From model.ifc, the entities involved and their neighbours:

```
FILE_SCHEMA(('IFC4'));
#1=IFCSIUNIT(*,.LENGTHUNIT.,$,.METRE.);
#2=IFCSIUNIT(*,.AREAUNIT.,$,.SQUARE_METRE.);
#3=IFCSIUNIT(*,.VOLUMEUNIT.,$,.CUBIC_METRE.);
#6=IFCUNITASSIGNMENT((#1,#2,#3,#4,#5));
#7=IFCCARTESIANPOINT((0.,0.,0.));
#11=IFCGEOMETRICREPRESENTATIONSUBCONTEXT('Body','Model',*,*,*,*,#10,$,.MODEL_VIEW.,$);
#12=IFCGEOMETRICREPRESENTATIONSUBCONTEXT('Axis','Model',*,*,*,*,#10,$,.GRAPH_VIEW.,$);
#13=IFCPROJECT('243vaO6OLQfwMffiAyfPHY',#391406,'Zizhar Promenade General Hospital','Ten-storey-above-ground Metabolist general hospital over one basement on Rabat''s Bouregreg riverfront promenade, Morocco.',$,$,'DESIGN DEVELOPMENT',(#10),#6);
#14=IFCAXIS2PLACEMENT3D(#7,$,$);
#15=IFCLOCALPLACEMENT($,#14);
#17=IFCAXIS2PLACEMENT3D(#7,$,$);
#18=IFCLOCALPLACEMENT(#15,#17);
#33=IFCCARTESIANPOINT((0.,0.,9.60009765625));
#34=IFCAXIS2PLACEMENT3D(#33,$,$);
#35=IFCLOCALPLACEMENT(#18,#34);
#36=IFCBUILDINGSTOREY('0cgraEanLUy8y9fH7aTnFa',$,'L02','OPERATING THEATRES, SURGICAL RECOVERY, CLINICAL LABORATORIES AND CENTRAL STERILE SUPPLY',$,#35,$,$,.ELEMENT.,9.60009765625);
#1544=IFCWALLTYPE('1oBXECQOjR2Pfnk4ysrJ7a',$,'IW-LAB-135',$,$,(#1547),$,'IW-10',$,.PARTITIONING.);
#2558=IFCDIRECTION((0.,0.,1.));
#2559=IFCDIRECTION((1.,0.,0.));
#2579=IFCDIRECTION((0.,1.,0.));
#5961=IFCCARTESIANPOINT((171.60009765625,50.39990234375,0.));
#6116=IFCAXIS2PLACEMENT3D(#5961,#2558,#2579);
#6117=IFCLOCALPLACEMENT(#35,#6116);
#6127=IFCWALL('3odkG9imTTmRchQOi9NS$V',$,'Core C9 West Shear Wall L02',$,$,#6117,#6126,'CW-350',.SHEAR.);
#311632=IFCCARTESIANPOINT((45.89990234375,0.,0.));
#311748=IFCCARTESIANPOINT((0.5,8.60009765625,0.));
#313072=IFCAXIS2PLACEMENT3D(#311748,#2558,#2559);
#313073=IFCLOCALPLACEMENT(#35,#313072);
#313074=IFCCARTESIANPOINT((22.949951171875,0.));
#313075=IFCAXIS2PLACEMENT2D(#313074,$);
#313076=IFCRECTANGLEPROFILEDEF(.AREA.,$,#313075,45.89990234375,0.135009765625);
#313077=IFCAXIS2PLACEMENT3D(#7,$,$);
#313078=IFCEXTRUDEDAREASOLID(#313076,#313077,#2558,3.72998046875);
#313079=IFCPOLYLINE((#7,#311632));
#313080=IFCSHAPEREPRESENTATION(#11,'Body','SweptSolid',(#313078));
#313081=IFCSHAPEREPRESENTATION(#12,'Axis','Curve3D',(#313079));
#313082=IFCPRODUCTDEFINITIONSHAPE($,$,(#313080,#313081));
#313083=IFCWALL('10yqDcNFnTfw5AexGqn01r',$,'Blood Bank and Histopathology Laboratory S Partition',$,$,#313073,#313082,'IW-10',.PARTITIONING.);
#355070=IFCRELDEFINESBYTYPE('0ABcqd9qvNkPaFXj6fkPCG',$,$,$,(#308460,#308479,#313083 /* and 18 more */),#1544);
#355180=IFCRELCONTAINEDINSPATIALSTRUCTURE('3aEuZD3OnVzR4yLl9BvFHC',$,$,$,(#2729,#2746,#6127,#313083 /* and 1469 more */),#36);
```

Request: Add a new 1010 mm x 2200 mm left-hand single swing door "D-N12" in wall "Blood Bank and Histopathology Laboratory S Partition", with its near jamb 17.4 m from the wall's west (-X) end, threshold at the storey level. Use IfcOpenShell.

```python
import numpy as np
import ifcopenshell
import ifcopenshell.api.feature
import ifcopenshell.api.geometry
import ifcopenshell.api.root
import ifcopenshell.api.spatial
import ifcopenshell.geom
import ifcopenshell.util.element
import ifcopenshell.util.placement
import ifcopenshell.util.representation
import ifcopenshell.util.shape
import ifcopenshell.util.unit

model = ifcopenshell.open("model.ifc")
unit_scale = ifcopenshell.util.unit.calculate_unit_scale(model)
settings = ifcopenshell.geom.settings()


def volume(element):
    """Net volume in cubic metres, openings subtracted."""
    shape = ifcopenshell.geom.create_shape(settings, element)
    return ifcopenshell.util.shape.get_volume(shape.geometry)


wall = model.by_guid("10yqDcNFnTfw5AexGqn01r")
storey = ifcopenshell.util.element.get_container(wall, ifc_class="IfcBuildingStorey")
context = ifcopenshell.util.representation.get_context(model, "Model", "Body", "MODEL_VIEW")
before = volume(wall)

width, height, from_end, sill = 1.01, 2.2, 17.4, 0.0  # metres

# The wall runs along its own X axis, and the end named is its -X end.
wall_shape = ifcopenshell.geom.create_shape(settings, wall)
x, y, z = ifcopenshell.util.shape.get_vertices(wall_shape.geometry).T
start = x.min() + from_end
face, thickness = float(y.min()), float(y.max() - y.min())
wall_matrix = ifcopenshell.util.placement.get_local_placement(wall.ObjectPlacement)
level = ifcopenshell.util.placement.get_local_placement(storey.ObjectPlacement)[2, 3]


def in_wall(x, y):
    """Placement at x, y metres in the wall's axes, at sill height."""
    matrix = wall_matrix.copy()
    matrix[:, 3] = wall_matrix @ np.array([x / unit_scale, y / unit_scale, 0.0, 1.0])
    matrix[2, 3] = level + sill / unit_scale
    return matrix


# Opening: a box that overshoots both wall faces by 50 mm.
opening = ifcopenshell.api.root.create_entity(model, ifc_class="IfcOpeningElement", predefined_type="OPENING")
box = ifcopenshell.api.geometry.add_wall_representation(
    model, context=context, length=width, height=height, thickness=thickness + 0.1
)
ifcopenshell.api.geometry.assign_representation(model, product=opening, representation=box)
ifcopenshell.api.geometry.edit_object_placement(model, product=opening, matrix=in_wall(start, face - 0.05), is_si=False)
ifcopenshell.api.feature.add_feature(model, feature=opening, element=wall)

door = ifcopenshell.api.root.create_entity(model, ifc_class="IfcDoor", name="D-N12", predefined_type="DOOR")
door.OverallWidth, door.OverallHeight = width / unit_scale, height / unit_scale
door.OperationType = "SINGLE_SWING_LEFT"
body = ifcopenshell.api.geometry.add_door_representation(
    model,
    context=context,
    overall_width=door.OverallWidth,
    overall_height=door.OverallHeight,
    operation_type="SINGLE_SWING_LEFT",
    lining_properties={"LiningDepth": thickness / unit_scale, "ThresholdDepth": thickness / unit_scale},
)
ifcopenshell.api.geometry.assign_representation(model, product=door, representation=body)
ifcopenshell.api.spatial.assign_container(model, products=[door], relating_structure=storey)
ifcopenshell.api.feature.add_filling(model, opening=opening, element=door)

# The lining spans the wall, so the door starts at the wall face.
ifcopenshell.api.geometry.edit_object_placement(model, product=door, matrix=in_wall(start, face), is_si=False)

after = volume(wall)

print(f"wall volume {before:.3f} -> {after:.3f} m3")

model.write("model_v2.ifc")
```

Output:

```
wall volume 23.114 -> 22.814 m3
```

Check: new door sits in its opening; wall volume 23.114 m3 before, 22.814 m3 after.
